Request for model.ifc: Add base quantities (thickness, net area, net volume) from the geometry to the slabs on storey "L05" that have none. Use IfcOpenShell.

First a look at what the model holds.

```python
import ifcopenshell
import ifcopenshell.util.element
import ifcopenshell.util.unit

model = ifcopenshell.open("model.ifc")
print(model.schema)
for unit_type in ("LENGTHUNIT", "AREAUNIT", "VOLUMEUNIT"):
    print(unit_type, ifcopenshell.util.unit.calculate_unit_scale(model, unit_type))
storey = next(s for s in model.by_type("IfcBuildingStorey") if s.Name == "L05")
slabs = [e for e in ifcopenshell.util.element.get_decomposition(storey) if e.is_a("IfcSlab")]
for e in sorted(slabs, key=lambda e: e.id()):
    print(e.id(), e.is_a(), e.Name, list(ifcopenshell.util.element.get_psets(e, qtos_only=True)), sep=" | ")
```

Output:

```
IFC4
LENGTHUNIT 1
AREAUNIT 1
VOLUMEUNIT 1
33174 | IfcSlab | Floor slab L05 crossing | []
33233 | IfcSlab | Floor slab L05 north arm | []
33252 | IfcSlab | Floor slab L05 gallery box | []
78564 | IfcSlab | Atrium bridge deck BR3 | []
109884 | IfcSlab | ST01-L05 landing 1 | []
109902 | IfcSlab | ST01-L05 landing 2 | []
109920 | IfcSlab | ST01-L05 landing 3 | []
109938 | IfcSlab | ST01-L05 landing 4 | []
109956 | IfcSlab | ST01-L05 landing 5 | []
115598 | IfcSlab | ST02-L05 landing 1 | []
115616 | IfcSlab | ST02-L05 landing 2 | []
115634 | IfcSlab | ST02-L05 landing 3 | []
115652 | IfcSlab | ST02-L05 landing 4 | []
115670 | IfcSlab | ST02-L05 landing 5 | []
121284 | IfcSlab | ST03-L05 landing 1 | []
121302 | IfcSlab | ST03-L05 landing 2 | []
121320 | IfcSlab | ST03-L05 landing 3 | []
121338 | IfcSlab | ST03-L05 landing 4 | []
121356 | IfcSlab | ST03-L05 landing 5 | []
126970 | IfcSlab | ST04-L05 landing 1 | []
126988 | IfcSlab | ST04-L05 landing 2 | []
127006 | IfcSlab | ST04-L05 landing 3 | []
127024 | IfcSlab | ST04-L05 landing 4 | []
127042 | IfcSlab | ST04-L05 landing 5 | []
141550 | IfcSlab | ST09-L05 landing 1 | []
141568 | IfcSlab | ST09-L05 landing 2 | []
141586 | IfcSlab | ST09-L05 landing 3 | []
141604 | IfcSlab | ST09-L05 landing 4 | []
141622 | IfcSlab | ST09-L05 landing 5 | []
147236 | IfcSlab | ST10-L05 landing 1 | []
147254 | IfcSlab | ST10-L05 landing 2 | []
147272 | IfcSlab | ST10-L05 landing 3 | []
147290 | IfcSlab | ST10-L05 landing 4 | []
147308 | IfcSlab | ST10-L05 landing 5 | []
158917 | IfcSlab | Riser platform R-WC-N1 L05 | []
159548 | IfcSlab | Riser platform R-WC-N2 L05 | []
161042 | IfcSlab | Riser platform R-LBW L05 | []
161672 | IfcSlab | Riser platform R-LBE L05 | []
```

```python
import ifcopenshell
import ifcopenshell.api.pset
import ifcopenshell.geom
import ifcopenshell.util.element
import ifcopenshell.util.shape
import ifcopenshell.util.unit

model = ifcopenshell.open("model.ifc")
unit_scale = ifcopenshell.util.unit.calculate_unit_scale(model)
area_scale = ifcopenshell.util.unit.calculate_unit_scale(model, "AREAUNIT")
volume_scale = ifcopenshell.util.unit.calculate_unit_scale(model, "VOLUMEUNIT")
settings = ifcopenshell.geom.settings()

storey = next(s for s in model.by_type("IfcBuildingStorey") if s.Name == "L05")
slabs = [e for e in ifcopenshell.util.element.get_decomposition(storey) if e.is_a("IfcSlab")]

for e in sorted(slabs, key=lambda e: e.id()):
    if ifcopenshell.util.element.get_psets(e, qtos_only=True, should_inherit=False):
        continue
    # Geometry comes back in metres, in the element's own axes.
    shape = ifcopenshell.geom.create_shape(settings, e)
    values = {
        "Width": ifcopenshell.util.shape.get_z(shape.geometry) / unit_scale,
        "NetArea": ifcopenshell.util.shape.get_footprint_area(shape.geometry) / area_scale,
        "NetVolume": ifcopenshell.util.shape.get_volume(shape.geometry) / volume_scale,
    }
    qto = ifcopenshell.api.pset.add_qto(model, product=e, name="Qto_SlabBaseQuantities")
    ifcopenshell.api.pset.edit_qto(model, qto=qto, properties=values)
    print(e.id(), {k: round(v, 3) for k, v in values.items()})

model.write("model_updated.ifc")
```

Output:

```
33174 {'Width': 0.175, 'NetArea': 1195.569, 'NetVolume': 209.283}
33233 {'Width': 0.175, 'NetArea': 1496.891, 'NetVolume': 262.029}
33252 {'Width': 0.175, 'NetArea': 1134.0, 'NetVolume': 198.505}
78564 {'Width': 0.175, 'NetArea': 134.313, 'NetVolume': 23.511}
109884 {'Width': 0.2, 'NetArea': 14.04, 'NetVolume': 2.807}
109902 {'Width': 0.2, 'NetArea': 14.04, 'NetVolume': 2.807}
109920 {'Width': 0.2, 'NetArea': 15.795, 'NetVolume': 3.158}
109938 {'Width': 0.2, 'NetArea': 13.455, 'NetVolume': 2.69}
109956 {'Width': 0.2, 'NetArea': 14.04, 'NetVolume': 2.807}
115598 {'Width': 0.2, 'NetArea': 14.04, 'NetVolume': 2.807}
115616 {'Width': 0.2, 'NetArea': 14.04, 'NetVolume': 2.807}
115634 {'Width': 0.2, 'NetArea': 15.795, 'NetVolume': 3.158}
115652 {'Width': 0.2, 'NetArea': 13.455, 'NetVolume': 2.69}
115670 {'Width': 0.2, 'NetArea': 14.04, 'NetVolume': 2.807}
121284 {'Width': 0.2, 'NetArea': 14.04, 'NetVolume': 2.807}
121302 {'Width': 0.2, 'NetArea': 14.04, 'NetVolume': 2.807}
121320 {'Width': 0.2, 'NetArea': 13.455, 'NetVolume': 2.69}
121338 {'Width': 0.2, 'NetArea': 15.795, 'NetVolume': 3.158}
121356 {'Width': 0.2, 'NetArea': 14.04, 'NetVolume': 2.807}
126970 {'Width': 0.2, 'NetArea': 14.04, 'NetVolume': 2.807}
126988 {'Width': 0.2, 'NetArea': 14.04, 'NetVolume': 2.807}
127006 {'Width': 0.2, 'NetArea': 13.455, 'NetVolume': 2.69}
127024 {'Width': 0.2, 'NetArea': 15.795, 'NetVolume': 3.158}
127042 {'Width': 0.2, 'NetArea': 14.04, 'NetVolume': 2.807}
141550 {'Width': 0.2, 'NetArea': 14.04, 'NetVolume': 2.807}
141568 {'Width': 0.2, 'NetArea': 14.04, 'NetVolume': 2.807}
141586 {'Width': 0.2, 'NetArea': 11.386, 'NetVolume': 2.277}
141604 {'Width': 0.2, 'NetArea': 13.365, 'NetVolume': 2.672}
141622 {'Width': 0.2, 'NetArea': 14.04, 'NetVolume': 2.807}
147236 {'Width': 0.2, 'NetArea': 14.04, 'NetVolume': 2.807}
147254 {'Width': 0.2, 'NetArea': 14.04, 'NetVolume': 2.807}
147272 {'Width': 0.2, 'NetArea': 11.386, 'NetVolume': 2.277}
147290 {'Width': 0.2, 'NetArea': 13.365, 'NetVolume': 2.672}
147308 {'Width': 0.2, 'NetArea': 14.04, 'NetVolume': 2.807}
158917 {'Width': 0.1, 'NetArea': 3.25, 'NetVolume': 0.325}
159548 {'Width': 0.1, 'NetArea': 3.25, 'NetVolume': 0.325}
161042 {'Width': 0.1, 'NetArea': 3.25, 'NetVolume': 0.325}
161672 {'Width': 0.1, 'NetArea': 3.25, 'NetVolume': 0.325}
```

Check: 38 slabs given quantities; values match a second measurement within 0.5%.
